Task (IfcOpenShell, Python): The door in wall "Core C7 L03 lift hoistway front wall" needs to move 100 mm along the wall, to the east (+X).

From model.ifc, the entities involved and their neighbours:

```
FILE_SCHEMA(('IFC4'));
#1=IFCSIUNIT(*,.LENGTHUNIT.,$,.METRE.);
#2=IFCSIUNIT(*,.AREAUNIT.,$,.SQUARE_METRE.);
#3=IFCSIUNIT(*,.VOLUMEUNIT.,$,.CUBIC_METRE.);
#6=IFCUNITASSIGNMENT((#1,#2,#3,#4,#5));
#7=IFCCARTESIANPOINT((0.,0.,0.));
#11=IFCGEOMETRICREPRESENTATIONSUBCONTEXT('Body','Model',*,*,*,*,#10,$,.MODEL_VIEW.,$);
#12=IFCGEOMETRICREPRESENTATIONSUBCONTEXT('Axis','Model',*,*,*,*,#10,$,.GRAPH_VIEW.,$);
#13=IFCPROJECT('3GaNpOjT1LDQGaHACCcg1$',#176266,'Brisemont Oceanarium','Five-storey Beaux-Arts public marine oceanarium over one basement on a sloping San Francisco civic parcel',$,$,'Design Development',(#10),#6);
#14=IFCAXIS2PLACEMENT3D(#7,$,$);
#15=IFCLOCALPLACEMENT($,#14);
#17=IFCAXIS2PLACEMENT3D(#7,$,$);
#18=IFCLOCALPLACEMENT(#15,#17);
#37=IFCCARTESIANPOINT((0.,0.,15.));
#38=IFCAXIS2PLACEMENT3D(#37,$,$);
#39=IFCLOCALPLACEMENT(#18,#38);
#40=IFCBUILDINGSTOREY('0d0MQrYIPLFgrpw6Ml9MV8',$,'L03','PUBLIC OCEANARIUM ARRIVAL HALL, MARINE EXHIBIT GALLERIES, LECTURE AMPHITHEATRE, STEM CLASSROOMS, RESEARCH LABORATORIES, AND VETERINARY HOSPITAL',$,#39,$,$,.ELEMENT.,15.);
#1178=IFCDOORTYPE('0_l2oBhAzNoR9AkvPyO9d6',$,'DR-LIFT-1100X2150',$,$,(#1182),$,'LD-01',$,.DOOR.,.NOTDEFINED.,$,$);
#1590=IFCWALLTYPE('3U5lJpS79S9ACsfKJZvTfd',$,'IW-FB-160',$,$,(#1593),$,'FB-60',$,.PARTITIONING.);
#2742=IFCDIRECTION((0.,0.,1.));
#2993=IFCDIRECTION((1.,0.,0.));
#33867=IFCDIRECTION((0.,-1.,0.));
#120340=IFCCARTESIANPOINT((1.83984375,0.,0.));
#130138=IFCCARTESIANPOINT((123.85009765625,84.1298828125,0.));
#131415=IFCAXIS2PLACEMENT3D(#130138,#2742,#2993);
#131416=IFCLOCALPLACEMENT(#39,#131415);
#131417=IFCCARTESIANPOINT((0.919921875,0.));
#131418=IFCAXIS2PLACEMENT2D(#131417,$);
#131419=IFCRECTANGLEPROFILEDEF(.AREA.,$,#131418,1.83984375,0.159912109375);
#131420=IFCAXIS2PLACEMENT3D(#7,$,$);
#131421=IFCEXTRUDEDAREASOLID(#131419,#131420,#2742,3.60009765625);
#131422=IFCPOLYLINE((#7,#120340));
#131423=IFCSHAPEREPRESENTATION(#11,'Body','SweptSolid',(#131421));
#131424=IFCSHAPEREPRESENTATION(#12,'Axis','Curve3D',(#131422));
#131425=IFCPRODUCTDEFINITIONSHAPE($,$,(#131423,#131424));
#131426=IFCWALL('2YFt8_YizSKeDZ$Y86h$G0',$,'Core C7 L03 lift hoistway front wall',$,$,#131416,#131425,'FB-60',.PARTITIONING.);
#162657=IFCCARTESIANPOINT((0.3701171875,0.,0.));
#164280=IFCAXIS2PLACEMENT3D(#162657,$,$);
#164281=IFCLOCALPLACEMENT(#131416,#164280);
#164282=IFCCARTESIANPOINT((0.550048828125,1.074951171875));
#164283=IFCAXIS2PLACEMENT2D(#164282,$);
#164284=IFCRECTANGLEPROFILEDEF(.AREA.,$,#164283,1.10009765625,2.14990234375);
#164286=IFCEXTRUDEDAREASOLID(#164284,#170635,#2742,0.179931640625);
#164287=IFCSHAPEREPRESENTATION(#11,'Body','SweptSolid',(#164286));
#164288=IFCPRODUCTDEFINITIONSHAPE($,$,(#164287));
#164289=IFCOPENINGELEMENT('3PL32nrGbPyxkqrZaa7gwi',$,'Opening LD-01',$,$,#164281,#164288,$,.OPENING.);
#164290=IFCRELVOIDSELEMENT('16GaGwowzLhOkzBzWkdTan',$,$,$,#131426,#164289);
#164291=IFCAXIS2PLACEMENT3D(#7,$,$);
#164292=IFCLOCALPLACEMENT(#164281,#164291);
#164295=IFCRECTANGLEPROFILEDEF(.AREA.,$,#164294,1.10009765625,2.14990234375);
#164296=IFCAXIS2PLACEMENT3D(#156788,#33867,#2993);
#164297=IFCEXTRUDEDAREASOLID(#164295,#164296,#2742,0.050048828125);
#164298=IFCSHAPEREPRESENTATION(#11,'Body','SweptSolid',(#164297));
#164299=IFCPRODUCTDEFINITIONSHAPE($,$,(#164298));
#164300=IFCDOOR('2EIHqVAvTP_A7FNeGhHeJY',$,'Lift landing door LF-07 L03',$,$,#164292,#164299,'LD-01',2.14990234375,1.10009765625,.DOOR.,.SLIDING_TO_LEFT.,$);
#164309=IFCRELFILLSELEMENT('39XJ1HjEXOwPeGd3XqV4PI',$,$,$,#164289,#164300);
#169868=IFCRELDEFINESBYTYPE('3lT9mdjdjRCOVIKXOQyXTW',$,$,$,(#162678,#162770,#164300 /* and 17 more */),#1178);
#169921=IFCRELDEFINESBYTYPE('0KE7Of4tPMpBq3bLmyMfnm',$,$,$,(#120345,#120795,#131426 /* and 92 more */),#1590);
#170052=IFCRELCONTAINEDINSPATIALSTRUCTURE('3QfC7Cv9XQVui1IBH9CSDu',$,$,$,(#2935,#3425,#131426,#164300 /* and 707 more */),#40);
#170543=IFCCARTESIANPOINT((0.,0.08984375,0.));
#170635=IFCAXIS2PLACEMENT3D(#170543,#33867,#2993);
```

```python
import ifcopenshell
import ifcopenshell.api.geometry
import ifcopenshell.util.placement

model = ifcopenshell.open("model.ifc")

door = model.by_guid("2EIHqVAvTP_A7FNeGhHeJY")
opening = door.FillsVoids[0].RelatingOpeningElement
wall = opening.VoidsElements[0].RelatingBuildingElement

wall_matrix = ifcopenshell.util.placement.get_local_placement(wall.ObjectPlacement)
shift = wall_matrix[:3, 0] * 0.1
before = ifcopenshell.util.placement.get_local_placement(door.ObjectPlacement)[:3, 3].copy()

# The door is placed relative to its opening, so it follows when the opening moves.
matrix = ifcopenshell.util.placement.get_local_placement(opening.ObjectPlacement)
matrix[:3, 3] += shift
ifcopenshell.api.geometry.edit_object_placement(
    model, product=opening, matrix=matrix, is_si=False, should_transform_children=True
)

after = ifcopenshell.util.placement.get_local_placement(door.ObjectPlacement)[:3, 3]
print("door moved by", (after - before).round(3) + 0.0)

model.write("model_v2.ifc")
```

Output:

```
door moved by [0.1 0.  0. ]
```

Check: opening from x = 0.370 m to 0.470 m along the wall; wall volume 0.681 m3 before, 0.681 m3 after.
